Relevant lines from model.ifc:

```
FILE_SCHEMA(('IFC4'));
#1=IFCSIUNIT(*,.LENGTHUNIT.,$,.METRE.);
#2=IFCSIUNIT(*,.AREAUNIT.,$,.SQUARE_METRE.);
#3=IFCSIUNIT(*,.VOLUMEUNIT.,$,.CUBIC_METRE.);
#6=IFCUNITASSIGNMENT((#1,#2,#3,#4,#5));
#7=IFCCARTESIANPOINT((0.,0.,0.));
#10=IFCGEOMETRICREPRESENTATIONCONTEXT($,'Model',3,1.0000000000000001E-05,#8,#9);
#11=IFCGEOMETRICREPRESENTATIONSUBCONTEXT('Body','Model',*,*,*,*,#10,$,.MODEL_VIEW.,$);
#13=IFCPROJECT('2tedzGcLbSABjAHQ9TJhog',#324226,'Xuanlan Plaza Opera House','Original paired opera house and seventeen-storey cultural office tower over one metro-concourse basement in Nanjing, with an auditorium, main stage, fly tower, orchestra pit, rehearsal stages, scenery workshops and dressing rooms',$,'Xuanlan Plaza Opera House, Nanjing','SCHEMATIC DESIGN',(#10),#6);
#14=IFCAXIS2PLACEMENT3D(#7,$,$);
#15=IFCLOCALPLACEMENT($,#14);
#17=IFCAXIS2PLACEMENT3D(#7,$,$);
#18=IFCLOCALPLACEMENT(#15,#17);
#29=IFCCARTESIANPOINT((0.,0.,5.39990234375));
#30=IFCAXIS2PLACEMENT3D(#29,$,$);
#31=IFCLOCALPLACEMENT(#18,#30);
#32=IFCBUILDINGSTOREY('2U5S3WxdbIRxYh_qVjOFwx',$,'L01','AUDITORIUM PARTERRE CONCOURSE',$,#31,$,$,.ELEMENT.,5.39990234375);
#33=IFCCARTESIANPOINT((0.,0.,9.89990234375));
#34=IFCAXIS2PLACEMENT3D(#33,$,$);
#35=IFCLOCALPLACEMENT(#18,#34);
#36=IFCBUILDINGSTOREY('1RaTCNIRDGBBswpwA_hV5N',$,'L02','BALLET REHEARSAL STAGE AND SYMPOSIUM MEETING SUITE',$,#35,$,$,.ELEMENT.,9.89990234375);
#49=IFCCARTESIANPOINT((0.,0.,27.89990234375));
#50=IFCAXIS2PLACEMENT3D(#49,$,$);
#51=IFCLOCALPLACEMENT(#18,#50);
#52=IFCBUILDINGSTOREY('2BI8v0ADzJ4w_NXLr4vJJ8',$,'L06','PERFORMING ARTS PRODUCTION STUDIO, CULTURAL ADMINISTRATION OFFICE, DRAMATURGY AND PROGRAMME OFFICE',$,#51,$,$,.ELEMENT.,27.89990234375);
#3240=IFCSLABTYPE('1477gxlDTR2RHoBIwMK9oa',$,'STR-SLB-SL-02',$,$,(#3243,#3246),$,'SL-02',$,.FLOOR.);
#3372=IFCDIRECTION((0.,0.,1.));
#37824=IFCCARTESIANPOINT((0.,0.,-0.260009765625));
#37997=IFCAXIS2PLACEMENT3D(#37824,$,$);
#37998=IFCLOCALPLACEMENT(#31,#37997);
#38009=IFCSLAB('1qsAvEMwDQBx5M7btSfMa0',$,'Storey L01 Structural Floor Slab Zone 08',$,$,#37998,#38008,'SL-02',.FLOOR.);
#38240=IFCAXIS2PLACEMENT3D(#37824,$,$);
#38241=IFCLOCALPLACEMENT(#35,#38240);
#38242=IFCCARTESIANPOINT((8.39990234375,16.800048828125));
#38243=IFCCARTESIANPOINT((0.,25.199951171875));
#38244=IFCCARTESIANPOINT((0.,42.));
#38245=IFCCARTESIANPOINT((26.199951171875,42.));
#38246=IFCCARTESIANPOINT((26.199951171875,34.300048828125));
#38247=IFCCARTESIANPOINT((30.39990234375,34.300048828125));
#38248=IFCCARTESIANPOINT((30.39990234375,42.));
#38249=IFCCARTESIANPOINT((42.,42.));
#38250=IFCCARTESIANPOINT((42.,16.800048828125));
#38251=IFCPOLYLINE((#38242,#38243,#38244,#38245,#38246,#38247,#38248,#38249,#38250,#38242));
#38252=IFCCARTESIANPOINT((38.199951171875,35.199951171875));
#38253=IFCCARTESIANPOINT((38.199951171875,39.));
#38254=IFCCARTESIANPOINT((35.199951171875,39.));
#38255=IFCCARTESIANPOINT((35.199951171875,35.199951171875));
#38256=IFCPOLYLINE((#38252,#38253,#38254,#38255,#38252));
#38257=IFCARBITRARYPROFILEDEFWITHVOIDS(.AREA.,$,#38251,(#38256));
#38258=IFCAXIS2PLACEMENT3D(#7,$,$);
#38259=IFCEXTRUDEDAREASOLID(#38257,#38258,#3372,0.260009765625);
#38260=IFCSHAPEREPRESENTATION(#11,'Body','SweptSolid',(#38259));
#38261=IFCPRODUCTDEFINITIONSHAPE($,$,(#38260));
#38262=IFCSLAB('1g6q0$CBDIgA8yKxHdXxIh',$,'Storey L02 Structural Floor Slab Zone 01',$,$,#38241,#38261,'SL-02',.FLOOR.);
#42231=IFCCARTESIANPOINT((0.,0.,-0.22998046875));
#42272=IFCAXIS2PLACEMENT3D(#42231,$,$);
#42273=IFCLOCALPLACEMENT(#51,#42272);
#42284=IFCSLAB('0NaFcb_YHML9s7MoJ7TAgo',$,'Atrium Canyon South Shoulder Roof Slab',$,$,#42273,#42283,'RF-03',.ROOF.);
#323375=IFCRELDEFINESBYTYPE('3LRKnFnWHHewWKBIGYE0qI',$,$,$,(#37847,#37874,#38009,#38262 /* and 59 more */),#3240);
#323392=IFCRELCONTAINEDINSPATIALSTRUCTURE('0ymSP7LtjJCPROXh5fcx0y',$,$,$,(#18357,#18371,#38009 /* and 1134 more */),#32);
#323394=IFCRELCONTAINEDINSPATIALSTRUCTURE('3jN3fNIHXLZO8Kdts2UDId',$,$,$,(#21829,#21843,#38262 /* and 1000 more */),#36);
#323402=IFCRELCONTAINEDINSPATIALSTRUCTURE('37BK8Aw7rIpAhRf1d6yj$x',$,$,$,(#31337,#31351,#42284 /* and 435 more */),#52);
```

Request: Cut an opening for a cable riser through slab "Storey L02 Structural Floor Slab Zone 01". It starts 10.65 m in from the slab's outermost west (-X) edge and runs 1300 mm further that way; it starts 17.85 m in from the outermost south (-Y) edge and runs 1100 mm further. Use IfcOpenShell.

```python
import numpy as np
import ifcopenshell
import ifcopenshell.api.feature
import ifcopenshell.api.geometry
import ifcopenshell.api.root
import ifcopenshell.geom
import ifcopenshell.util.placement
import ifcopenshell.util.representation
import ifcopenshell.util.shape
import ifcopenshell.util.unit

model = ifcopenshell.open("model.ifc")
unit_scale = ifcopenshell.util.unit.calculate_unit_scale(model)
settings = ifcopenshell.geom.settings()


def volume(element):
    """Net volume in cubic metres, openings subtracted."""
    shape = ifcopenshell.geom.create_shape(settings, element)
    return ifcopenshell.util.shape.get_volume(shape.geometry)


slab = model.by_guid("1g6q0$CBDIgA8yKxHdXxIh")
before = volume(slab)

# Extent in the slab's own axes, in metres. The edges named are its -X and -Y sides.
slab_shape = ifcopenshell.geom.create_shape(settings, slab)
vertices = ifcopenshell.util.shape.get_vertices(slab_shape.geometry)
x_min, y_min, bottom = vertices.min(axis=0)
top = vertices[:, 2].max()

opening = ifcopenshell.api.root.create_entity(model, ifc_class="IfcOpeningElement", name="Cable riser opening", predefined_type="OPENING")
context = ifcopenshell.util.representation.get_context(model, "Model", "Body", "MODEL_VIEW")
width, depth = 1.3, 1.1
outline = [(0.0, 0.0), (width, 0.0), (width, depth), (0.0, depth), (0.0, 0.0)]
# Overshoot both faces by 50 mm so the cut is clean.
shape = ifcopenshell.api.geometry.add_slab_representation(
    model, context=context, depth=top - bottom + 0.1, polyline=outline
)
ifcopenshell.api.geometry.assign_representation(model, product=opening, representation=shape)

matrix = ifcopenshell.util.placement.get_local_placement(slab.ObjectPlacement)
matrix[:, 3] = matrix @ np.append(np.array([x_min + 10.65, y_min + 17.85, bottom - 0.05]) / unit_scale, 1.0)
ifcopenshell.api.geometry.edit_object_placement(model, product=opening, matrix=matrix, is_si=False)
ifcopenshell.api.feature.add_feature(model, feature=opening, element=slab)

after = volume(slab)

print(f"slab volume {before:.3f} -> {after:.3f} m3")

model.write("model_v2.ifc")
```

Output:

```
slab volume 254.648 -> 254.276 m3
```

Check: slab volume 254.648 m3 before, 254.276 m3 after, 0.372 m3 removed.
